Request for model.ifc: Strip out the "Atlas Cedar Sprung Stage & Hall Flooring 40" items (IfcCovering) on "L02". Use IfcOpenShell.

First a look at what the model holds.

```python
import ifcopenshell
import ifcopenshell.util.element

model = ifcopenshell.open("model.ifc")
print(model.schema)
storey = next(s for s in model.by_type("IfcBuildingStorey") if s.Name == "L02")
coverings = [e for e in ifcopenshell.util.element.get_decomposition(storey) if e.is_a("IfcCovering")]
seen = {}
for e in coverings:
    element_type = ifcopenshell.util.element.get_type(e)
    name = element_type.Name if element_type not in (None, e) else None
    seen[name] = seen.get(name, 0) + 1
for name, count in sorted(seen.items(), key=str):
    print(count, "x", name)
```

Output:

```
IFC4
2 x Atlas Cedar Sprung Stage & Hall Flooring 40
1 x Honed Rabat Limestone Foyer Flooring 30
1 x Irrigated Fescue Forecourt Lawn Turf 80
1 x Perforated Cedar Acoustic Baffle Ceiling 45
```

```python
import ifcopenshell
import ifcopenshell.api.root
import ifcopenshell.util.element

model = ifcopenshell.open("model.ifc")

storey = next(s for s in model.by_type("IfcBuildingStorey") if s.Name == "L02")
coverings = [e for e in ifcopenshell.util.element.get_decomposition(storey) if e.is_a("IfcCovering")]
targets = [e for e in coverings if (t := ifcopenshell.util.element.get_type(e)) not in (None, e) and t.Name == "Atlas Cedar Sprung Stage & Hall Flooring 40"]

for e in targets:
    ifcopenshell.api.root.remove_product(model, product=e)
print(len(targets), "removed")

model.write("model_v2.ifc")
```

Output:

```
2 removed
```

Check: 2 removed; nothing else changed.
